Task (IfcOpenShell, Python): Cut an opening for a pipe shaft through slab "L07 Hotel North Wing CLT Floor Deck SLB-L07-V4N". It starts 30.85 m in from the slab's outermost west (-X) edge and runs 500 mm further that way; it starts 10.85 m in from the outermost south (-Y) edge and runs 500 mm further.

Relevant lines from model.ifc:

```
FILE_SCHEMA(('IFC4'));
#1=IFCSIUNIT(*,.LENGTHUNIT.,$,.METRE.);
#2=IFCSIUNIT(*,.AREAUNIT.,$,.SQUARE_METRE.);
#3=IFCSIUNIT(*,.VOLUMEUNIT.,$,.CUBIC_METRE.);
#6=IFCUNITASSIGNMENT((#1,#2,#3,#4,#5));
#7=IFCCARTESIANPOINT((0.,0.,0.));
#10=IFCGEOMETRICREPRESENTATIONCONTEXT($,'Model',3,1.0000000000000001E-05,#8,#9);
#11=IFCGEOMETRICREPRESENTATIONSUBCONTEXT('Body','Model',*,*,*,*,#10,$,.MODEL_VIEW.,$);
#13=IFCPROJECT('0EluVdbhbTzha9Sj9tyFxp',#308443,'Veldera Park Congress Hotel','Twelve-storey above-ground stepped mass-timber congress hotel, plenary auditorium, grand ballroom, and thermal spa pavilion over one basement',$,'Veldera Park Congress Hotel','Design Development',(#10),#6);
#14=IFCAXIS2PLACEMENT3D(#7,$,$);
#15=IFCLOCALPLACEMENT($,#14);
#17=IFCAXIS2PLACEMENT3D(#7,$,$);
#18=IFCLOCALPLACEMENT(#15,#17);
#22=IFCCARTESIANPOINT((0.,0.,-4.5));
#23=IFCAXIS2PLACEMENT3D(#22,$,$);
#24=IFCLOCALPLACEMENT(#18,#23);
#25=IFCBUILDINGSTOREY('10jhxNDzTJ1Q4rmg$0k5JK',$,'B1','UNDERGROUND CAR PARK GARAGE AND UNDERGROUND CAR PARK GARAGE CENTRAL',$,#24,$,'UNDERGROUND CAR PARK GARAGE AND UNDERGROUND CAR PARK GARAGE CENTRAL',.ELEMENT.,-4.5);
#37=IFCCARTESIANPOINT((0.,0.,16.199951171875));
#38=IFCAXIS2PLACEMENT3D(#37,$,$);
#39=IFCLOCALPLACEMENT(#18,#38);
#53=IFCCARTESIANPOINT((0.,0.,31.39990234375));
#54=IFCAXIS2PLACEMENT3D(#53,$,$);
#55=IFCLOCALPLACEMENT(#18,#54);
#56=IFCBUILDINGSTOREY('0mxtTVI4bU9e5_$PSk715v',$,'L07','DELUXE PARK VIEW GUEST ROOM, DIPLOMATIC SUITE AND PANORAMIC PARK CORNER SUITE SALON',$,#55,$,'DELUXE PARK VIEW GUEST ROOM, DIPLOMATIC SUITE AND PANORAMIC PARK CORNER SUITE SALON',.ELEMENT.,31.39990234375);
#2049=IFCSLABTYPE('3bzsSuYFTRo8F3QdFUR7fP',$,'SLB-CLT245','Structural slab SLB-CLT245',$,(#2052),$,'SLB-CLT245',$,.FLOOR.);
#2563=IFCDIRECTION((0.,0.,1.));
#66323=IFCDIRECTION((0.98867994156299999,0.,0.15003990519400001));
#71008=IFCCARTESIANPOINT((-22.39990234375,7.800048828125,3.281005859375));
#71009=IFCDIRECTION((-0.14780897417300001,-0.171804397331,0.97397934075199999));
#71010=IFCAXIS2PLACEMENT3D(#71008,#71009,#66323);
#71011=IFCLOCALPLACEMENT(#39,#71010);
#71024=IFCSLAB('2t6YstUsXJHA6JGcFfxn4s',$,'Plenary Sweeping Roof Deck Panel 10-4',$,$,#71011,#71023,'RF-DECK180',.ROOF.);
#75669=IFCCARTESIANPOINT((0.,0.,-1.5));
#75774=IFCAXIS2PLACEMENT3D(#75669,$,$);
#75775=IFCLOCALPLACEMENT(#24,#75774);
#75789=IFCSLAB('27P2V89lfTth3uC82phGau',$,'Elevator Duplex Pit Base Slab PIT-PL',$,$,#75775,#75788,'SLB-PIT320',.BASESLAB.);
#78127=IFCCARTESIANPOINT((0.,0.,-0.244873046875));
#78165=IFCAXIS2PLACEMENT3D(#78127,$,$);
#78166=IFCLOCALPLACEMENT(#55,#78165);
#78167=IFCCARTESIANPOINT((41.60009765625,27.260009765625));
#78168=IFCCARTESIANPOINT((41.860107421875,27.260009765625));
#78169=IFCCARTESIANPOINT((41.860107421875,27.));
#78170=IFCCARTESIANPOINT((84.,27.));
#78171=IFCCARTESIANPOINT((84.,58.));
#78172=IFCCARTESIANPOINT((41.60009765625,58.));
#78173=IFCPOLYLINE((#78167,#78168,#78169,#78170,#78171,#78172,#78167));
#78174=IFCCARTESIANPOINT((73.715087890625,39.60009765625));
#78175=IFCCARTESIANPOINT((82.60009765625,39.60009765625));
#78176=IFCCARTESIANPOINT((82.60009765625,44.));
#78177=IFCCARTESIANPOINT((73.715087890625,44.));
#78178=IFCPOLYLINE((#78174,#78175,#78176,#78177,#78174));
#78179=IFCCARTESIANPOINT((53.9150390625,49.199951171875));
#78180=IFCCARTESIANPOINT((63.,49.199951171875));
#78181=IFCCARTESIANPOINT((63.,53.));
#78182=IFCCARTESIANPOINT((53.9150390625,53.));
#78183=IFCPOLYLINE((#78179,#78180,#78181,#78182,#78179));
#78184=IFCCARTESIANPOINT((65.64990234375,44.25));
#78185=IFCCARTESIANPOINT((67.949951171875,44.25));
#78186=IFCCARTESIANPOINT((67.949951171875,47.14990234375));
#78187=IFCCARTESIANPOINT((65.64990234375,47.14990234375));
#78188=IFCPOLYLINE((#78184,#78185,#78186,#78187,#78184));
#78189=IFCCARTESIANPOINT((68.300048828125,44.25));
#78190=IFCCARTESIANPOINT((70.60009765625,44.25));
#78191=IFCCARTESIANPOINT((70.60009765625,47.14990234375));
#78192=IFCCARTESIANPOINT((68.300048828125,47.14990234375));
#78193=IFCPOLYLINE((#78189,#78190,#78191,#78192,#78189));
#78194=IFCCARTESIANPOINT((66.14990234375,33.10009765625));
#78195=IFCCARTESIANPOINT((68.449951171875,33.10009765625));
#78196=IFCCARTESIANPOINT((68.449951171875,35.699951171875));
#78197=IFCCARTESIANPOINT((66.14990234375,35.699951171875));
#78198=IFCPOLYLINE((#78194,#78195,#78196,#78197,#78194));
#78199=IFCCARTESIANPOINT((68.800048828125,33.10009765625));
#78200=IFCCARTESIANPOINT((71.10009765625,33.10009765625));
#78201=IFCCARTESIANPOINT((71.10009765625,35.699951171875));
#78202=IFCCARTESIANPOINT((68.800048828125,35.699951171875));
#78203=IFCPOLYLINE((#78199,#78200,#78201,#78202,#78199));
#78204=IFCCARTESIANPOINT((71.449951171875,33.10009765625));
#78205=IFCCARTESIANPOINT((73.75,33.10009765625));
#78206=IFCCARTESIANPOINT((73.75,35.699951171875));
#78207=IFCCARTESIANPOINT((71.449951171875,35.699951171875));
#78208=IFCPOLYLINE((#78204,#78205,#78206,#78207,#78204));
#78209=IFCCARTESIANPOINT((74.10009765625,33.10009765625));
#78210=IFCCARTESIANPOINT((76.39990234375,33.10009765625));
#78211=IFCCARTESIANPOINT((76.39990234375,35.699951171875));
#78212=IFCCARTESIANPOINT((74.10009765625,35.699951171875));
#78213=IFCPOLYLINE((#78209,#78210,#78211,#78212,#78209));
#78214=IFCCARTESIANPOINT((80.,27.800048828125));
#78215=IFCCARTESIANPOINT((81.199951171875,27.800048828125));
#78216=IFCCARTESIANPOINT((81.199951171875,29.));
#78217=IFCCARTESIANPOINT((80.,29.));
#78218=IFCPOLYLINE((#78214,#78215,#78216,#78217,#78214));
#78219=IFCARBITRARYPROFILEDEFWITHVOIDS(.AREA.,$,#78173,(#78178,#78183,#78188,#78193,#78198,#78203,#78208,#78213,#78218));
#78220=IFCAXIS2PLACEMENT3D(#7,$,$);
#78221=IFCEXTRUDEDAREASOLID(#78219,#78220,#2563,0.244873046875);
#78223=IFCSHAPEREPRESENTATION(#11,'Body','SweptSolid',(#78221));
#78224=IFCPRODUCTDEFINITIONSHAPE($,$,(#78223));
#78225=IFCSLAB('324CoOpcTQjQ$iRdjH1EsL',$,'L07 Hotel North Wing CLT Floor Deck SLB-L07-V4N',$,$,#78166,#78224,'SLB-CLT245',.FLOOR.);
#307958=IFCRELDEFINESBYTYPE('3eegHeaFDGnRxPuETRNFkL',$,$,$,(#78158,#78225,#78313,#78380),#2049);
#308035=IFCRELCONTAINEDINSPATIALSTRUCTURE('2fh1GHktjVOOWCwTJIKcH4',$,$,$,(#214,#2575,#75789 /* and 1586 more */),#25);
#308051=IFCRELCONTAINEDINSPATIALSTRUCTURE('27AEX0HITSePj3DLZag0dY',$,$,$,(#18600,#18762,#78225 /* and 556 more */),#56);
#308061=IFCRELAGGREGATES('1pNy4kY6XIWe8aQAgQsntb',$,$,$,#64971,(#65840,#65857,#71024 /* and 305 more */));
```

```python
import numpy as np
import ifcopenshell
import ifcopenshell.api.feature
import ifcopenshell.api.geometry
import ifcopenshell.api.root
import ifcopenshell.geom
import ifcopenshell.util.placement
import ifcopenshell.util.representation
import ifcopenshell.util.shape
import ifcopenshell.util.unit

model = ifcopenshell.open("model.ifc")
unit_scale = ifcopenshell.util.unit.calculate_unit_scale(model)
settings = ifcopenshell.geom.settings()


def volume(element):
    """Net volume in cubic metres, openings subtracted."""
    shape = ifcopenshell.geom.create_shape(settings, element)
    return ifcopenshell.util.shape.get_volume(shape.geometry)


slab = model.by_guid("324CoOpcTQjQ$iRdjH1EsL")
before = volume(slab)

# Extent in the slab's own axes, in metres. The edges named are its -X and -Y sides.
slab_shape = ifcopenshell.geom.create_shape(settings, slab)
vertices = ifcopenshell.util.shape.get_vertices(slab_shape.geometry)
x_min, y_min, bottom = vertices.min(axis=0)
top = vertices[:, 2].max()

opening = ifcopenshell.api.root.create_entity(model, ifc_class="IfcOpeningElement", name="Pipe shaft opening", predefined_type="OPENING")
context = ifcopenshell.util.representation.get_context(model, "Model", "Body", "MODEL_VIEW")
width, depth = 0.5, 0.5
outline = [(0.0, 0.0), (width, 0.0), (width, depth), (0.0, depth), (0.0, 0.0)]
# Overshoot both faces by 50 mm so the cut is clean.
shape = ifcopenshell.api.geometry.add_slab_representation(
    model, context=context, depth=top - bottom + 0.1, polyline=outline
)
ifcopenshell.api.geometry.assign_representation(model, product=opening, representation=shape)

matrix = ifcopenshell.util.placement.get_local_placement(slab.ObjectPlacement)
matrix[:, 3] = matrix @ np.append(np.array([x_min + 30.85, y_min + 10.85, bottom - 0.05]) / unit_scale, 1.0)
ifcopenshell.api.geometry.edit_object_placement(model, product=opening, matrix=matrix, is_si=False)
ifcopenshell.api.feature.add_feature(model, feature=opening, element=slab)

after = volume(slab)

print(f"slab volume {before:.3f} -> {after:.3f} m3")

model.write("model_rev.ifc")
```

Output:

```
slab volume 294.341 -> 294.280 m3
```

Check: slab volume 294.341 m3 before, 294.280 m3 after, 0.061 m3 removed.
